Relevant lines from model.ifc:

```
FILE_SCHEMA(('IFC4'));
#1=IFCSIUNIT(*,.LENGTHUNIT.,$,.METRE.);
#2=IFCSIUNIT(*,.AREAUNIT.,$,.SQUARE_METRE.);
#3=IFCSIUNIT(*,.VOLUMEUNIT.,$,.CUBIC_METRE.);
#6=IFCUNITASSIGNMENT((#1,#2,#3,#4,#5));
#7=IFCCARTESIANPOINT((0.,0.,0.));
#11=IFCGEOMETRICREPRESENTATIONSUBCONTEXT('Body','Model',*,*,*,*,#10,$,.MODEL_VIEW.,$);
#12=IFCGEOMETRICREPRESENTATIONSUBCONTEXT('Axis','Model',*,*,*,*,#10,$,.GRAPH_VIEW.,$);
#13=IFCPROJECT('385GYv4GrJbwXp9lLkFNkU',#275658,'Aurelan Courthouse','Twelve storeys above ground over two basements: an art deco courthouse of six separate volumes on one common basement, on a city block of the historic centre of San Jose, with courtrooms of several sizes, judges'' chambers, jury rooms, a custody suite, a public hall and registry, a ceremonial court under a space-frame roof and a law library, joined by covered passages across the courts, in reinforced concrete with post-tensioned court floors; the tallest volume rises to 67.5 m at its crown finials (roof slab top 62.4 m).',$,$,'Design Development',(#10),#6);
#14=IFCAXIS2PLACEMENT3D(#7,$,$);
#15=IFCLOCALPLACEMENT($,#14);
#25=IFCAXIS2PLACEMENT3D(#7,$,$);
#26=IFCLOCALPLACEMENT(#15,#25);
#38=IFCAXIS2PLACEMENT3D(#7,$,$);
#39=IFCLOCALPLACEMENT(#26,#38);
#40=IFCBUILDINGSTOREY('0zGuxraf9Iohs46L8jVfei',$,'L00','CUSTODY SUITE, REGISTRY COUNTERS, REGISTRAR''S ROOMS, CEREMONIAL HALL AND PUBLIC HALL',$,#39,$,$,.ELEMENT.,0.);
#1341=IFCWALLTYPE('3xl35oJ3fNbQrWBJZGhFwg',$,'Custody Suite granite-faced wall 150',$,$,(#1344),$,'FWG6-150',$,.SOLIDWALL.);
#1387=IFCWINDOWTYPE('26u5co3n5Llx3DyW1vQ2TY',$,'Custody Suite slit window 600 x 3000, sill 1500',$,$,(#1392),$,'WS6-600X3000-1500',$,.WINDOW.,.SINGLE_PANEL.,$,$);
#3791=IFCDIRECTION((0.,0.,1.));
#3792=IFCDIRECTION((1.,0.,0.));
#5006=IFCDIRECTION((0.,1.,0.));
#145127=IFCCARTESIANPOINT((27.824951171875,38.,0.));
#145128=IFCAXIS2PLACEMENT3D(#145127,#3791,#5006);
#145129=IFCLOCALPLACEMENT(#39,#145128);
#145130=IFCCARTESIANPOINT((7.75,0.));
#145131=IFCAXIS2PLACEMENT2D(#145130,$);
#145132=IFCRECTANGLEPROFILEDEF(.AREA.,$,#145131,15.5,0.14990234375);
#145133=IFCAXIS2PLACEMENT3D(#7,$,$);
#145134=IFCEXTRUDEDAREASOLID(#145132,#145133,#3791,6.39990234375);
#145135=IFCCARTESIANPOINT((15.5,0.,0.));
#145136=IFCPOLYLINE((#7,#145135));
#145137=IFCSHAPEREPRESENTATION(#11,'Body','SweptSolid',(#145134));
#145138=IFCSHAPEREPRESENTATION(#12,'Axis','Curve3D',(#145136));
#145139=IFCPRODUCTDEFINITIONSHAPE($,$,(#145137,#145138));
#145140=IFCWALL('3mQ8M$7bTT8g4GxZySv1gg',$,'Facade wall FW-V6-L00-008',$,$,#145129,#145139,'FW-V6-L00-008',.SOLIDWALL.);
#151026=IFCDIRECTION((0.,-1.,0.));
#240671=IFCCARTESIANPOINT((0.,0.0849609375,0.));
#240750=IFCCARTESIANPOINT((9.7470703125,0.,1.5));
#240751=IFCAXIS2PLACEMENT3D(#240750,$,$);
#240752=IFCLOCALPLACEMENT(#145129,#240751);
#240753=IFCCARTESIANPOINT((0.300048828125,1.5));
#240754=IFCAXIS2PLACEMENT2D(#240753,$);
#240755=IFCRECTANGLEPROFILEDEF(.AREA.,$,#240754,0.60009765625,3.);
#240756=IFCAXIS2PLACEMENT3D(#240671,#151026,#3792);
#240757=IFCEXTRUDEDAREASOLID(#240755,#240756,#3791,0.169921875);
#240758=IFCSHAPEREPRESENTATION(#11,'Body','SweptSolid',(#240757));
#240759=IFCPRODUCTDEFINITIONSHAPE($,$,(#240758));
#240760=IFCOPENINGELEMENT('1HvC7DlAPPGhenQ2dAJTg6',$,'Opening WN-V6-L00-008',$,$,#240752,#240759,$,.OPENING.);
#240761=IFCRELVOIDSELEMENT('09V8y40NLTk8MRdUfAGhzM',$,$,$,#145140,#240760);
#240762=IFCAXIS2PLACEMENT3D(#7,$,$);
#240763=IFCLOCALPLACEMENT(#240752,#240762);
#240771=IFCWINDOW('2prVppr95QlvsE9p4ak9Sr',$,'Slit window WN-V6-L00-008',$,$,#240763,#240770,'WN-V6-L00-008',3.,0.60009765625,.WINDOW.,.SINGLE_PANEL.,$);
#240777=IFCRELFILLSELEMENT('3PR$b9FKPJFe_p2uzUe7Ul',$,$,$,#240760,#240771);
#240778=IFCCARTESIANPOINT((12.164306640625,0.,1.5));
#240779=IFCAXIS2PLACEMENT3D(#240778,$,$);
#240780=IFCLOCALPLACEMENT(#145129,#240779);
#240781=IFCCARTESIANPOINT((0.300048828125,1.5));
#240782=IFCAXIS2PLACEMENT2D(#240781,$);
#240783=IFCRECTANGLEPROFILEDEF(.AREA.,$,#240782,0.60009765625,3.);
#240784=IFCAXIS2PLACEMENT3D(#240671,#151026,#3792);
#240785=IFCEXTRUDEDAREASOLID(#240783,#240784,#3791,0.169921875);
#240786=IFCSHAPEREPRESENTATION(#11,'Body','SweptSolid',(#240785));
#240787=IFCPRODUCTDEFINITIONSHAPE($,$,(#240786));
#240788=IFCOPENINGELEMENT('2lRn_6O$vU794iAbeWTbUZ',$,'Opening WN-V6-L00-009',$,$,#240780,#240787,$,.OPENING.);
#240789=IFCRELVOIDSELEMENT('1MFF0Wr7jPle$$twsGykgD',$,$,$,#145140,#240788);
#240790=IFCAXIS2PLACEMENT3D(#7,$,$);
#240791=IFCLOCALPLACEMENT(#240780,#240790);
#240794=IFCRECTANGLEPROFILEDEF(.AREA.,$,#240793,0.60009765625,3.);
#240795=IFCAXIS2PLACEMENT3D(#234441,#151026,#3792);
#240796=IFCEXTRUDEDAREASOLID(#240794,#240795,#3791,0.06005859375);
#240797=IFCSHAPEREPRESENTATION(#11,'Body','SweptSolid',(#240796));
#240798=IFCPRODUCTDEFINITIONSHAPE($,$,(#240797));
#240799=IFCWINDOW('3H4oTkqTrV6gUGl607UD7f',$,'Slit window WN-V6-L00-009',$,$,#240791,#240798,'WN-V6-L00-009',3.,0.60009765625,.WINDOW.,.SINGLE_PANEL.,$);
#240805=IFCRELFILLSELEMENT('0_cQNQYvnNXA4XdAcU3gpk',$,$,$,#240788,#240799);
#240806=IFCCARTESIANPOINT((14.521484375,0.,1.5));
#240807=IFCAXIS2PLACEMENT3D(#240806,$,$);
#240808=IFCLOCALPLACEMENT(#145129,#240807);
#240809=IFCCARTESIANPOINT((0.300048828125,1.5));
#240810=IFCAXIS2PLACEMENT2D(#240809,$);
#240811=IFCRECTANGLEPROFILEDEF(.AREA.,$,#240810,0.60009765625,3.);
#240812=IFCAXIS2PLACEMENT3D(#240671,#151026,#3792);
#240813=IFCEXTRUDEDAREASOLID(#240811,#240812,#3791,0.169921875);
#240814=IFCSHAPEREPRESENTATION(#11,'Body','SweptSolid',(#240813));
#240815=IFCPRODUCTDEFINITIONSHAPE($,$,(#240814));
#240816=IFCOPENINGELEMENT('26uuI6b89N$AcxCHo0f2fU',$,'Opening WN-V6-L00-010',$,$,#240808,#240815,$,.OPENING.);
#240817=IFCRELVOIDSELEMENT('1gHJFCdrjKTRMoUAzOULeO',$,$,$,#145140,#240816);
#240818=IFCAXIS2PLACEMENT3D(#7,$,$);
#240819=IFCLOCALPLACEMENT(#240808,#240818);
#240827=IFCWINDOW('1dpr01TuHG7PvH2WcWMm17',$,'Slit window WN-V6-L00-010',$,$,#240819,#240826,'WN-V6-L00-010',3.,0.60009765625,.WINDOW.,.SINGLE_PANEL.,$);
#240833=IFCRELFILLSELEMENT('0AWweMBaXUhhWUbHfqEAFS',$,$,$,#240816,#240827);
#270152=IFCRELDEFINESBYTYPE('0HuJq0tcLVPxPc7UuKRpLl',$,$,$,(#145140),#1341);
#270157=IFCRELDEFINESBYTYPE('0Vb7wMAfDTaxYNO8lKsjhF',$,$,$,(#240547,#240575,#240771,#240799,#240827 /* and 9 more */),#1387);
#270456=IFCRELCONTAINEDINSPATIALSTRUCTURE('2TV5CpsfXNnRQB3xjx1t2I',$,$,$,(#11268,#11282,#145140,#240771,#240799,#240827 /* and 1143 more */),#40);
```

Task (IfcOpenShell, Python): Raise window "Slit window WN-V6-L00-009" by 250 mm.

```python
import numpy as np
import ifcopenshell
import ifcopenshell.api.geometry
import ifcopenshell.util.placement
import ifcopenshell.util.unit

model = ifcopenshell.open("model.ifc")
unit_scale = ifcopenshell.util.unit.calculate_unit_scale(model)

window = model.by_guid("3H4oTkqTrV6gUGl607UD7f")
opening = window.FillsVoids[0].RelatingOpeningElement
dz = 0.25 / unit_scale

shift = np.array([0.0, 0.0, dz])
# The window is placed relative to its opening, so it follows when the opening moves.
matrix = ifcopenshell.util.placement.get_local_placement(opening.ObjectPlacement)
matrix[:3, 3] += shift
ifcopenshell.api.geometry.edit_object_placement(
    model, product=opening, matrix=matrix, is_si=False, should_transform_children=True
)

print(f"moved by {dz * unit_scale:+.3f} m")

model.write("model_edited.ifc")
```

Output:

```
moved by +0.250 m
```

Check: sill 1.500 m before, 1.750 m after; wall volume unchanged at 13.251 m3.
